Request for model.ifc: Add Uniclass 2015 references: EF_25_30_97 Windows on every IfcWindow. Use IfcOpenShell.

First a look at what the model holds.

```python
import ifcopenshell

model = ifcopenshell.open("model.ifc")
print(model.schema)
print("classifications:", [c.Name for c in model.by_type("IfcClassification")])
for ifc_class in ("IfcDoor", "IfcRoof", "IfcStair", "IfcWall", "IfcWindow"):
    print(ifc_class, len(model.by_type(ifc_class)))
```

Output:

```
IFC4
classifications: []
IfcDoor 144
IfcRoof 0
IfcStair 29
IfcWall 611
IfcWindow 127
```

```python
import ifcopenshell
import ifcopenshell.api.classification

model = ifcopenshell.open("model.ifc")

system = ifcopenshell.api.classification.add_classification(model, classification="Uniclass 2015")

codes = {
    "IfcWindow": ("EF_25_30_97", "Windows"),
}
for ifc_class, (code, name) in codes.items():
    products = model.by_type(ifc_class)
    ifcopenshell.api.classification.add_reference(
        model, products=products, classification=system, identification=code, name=name
    )
    print(code, len(products))

model.write("model_edited.ifc")
```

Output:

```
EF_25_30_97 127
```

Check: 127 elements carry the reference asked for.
